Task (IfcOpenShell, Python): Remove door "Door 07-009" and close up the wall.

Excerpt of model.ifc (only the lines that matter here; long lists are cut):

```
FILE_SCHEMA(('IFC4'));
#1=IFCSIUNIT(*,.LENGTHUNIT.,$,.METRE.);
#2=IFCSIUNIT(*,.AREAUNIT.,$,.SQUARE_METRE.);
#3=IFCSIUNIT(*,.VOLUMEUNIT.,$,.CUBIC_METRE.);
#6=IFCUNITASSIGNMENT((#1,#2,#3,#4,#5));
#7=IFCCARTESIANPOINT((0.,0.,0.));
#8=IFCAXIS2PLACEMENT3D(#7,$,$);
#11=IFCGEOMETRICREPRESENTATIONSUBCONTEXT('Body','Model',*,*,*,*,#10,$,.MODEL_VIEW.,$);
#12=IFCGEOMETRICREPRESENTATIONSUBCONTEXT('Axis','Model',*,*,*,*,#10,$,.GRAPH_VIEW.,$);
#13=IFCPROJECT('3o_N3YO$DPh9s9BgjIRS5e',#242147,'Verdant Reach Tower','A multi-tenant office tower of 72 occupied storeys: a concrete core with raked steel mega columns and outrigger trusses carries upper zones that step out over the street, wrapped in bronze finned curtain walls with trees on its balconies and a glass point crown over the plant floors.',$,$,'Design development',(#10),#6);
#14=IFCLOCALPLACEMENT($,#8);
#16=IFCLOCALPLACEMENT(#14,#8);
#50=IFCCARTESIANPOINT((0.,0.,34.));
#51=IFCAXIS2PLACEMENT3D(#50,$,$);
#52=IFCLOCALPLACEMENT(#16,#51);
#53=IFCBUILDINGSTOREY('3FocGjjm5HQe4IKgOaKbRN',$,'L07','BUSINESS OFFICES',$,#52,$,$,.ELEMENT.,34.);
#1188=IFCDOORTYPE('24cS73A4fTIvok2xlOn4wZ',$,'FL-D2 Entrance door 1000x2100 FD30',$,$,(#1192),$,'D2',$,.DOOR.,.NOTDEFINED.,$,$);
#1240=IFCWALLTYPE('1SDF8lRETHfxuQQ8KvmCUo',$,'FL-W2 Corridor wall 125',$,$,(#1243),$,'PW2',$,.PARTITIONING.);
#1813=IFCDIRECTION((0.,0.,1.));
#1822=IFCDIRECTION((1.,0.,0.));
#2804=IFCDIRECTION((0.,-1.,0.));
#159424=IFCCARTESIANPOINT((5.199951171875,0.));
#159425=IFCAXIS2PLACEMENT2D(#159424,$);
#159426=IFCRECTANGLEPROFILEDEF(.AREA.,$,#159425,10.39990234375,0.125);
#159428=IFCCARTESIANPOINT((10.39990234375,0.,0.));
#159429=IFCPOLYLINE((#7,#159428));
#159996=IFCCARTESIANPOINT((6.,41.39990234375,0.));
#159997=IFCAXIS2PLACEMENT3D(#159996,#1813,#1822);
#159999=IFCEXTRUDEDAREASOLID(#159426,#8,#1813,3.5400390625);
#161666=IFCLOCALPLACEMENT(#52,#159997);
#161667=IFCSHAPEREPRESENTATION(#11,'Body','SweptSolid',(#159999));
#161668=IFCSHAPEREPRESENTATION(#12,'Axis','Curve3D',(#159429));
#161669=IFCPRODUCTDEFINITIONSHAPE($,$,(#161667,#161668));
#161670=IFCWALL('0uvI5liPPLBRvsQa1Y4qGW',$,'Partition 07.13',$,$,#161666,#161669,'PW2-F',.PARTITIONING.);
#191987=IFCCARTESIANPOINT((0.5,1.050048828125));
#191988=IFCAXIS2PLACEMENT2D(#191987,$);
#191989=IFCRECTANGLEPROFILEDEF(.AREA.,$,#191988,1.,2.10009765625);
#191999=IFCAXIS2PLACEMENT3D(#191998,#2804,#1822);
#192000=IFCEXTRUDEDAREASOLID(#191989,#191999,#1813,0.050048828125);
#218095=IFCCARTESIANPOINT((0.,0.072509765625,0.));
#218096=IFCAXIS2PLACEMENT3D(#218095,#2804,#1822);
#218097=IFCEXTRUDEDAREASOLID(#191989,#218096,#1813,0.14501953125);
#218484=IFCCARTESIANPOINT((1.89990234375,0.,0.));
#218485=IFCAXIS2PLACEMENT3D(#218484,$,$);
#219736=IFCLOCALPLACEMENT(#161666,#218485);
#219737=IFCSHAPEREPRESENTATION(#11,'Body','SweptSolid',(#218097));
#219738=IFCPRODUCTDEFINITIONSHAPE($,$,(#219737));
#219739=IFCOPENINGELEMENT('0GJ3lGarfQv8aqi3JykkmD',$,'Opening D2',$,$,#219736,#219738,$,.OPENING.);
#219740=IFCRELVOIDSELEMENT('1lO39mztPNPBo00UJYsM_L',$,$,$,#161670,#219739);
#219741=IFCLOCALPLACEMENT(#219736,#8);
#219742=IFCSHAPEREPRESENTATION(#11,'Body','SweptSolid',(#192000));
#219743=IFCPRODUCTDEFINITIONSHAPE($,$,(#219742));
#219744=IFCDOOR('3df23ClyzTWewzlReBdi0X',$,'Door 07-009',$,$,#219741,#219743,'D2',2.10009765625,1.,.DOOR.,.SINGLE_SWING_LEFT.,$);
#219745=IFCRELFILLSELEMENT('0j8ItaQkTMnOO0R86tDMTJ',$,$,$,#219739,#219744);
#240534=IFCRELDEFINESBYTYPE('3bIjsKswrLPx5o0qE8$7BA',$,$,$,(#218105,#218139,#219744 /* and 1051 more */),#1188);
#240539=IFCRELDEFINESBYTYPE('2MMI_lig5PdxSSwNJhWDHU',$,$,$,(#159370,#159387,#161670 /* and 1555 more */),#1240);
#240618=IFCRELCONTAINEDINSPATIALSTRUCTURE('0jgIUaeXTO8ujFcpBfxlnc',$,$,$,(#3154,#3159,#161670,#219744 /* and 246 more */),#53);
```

```python
import ifcopenshell
import ifcopenshell.api.feature
import ifcopenshell.api.root
import ifcopenshell.geom
import ifcopenshell.util.shape

model = ifcopenshell.open("model.ifc")
settings = ifcopenshell.geom.settings()


def volume(element):
    """Net volume in cubic metres, openings subtracted."""
    shape = ifcopenshell.geom.create_shape(settings, element)
    return ifcopenshell.util.shape.get_volume(shape.geometry)


door = model.by_guid("3df23ClyzTWewzlReBdi0X")
opening = door.FillsVoids[0].RelatingOpeningElement
wall = opening.VoidsElements[0].RelatingBuildingElement
before = volume(wall)

ifcopenshell.api.root.remove_product(model, product=door)
ifcopenshell.api.feature.remove_feature(model, feature=opening)

after = volume(wall)

print(f"wall volume {before:.3f} -> {after:.3f} m3")

model.write("model-out.ifc")
```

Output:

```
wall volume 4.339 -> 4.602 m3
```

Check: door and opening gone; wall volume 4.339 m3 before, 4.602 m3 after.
